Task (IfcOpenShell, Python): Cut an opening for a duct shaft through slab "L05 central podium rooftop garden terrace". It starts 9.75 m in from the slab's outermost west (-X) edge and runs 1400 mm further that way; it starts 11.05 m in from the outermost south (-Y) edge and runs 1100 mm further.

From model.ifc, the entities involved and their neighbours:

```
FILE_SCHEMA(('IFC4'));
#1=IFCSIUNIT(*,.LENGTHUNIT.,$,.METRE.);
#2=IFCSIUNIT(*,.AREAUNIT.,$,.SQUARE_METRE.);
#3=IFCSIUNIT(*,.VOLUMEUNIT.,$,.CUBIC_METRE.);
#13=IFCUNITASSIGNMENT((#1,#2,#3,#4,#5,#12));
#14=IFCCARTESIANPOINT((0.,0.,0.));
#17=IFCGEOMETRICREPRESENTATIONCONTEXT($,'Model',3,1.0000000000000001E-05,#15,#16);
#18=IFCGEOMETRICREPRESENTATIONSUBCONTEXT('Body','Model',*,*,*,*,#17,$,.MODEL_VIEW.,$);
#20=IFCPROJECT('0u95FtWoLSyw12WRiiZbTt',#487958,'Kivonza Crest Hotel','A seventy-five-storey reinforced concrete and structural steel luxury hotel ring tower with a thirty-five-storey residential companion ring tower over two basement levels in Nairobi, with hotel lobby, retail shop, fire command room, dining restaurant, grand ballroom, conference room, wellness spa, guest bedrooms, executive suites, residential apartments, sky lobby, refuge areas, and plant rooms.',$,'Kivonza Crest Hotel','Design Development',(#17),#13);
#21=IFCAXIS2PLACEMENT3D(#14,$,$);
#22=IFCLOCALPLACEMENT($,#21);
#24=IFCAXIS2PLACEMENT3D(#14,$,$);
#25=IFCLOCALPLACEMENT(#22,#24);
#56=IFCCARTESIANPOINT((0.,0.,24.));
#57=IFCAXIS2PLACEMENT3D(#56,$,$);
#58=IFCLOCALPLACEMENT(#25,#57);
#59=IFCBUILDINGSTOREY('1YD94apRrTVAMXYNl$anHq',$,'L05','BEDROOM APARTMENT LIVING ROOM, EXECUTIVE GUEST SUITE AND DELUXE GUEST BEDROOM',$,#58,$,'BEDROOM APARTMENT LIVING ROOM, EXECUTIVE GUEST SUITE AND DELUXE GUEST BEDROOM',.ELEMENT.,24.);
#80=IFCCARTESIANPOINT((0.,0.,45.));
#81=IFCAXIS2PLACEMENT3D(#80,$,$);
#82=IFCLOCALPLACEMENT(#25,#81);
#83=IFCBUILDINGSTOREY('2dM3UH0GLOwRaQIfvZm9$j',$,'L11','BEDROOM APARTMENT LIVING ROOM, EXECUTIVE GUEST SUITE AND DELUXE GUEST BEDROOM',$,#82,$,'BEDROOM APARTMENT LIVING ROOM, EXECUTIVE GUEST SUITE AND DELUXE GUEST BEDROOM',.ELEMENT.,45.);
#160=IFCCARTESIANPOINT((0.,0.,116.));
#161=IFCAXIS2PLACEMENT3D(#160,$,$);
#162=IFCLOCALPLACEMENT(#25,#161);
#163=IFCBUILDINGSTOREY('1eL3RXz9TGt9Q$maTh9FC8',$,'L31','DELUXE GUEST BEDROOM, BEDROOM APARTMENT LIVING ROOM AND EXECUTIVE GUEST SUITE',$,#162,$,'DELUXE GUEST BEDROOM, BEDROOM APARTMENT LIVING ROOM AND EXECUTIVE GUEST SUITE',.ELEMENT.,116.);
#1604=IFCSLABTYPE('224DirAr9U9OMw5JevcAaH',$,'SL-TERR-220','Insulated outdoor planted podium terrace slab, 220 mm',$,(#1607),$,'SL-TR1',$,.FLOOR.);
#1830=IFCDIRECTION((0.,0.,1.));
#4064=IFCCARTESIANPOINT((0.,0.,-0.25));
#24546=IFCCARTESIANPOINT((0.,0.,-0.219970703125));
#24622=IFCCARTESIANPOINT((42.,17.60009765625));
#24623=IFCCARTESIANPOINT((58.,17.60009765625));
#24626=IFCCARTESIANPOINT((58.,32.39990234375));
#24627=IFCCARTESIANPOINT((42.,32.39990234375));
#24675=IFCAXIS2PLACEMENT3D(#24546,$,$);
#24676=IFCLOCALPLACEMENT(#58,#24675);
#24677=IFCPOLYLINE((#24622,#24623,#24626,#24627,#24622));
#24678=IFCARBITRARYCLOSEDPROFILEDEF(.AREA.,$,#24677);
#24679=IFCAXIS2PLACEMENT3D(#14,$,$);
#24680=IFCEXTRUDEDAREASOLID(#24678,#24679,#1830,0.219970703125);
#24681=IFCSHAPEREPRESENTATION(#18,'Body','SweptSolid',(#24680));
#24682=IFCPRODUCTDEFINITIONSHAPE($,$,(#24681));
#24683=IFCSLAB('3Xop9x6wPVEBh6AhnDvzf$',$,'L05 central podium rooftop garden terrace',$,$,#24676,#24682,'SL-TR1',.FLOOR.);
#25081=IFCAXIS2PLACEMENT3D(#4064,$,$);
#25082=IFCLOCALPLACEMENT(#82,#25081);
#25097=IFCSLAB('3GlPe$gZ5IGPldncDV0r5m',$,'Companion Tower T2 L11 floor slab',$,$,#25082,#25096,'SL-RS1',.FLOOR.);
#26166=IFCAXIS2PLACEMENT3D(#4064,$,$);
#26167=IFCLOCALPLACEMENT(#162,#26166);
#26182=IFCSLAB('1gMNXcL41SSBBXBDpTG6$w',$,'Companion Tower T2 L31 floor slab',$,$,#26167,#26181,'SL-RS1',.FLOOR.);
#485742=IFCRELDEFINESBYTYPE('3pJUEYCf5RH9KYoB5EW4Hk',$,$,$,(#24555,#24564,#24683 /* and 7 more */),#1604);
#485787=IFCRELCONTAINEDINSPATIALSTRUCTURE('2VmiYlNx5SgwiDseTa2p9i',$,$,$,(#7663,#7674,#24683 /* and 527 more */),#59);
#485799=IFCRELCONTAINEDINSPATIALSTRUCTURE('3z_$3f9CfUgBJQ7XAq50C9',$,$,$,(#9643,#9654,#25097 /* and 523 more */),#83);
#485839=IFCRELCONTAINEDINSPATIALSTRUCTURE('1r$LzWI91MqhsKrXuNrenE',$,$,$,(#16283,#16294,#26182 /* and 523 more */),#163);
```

```python
import numpy as np
import ifcopenshell
import ifcopenshell.api.feature
import ifcopenshell.api.geometry
import ifcopenshell.api.root
import ifcopenshell.geom
import ifcopenshell.util.placement
import ifcopenshell.util.representation
import ifcopenshell.util.shape
import ifcopenshell.util.unit

model = ifcopenshell.open("model.ifc")
unit_scale = ifcopenshell.util.unit.calculate_unit_scale(model)
settings = ifcopenshell.geom.settings()


def volume(element):
    """Net volume in cubic metres, openings subtracted."""
    shape = ifcopenshell.geom.create_shape(settings, element)
    return ifcopenshell.util.shape.get_volume(shape.geometry)


slab = model.by_guid("3Xop9x6wPVEBh6AhnDvzf$")
before = volume(slab)

# Extent in the slab's own axes, in metres. The edges named are its -X and -Y sides.
slab_shape = ifcopenshell.geom.create_shape(settings, slab)
vertices = ifcopenshell.util.shape.get_vertices(slab_shape.geometry)
x_min, y_min, bottom = vertices.min(axis=0)
top = vertices[:, 2].max()

opening = ifcopenshell.api.root.create_entity(model, ifc_class="IfcOpeningElement", name="Duct shaft opening", predefined_type="OPENING")
context = ifcopenshell.util.representation.get_context(model, "Model", "Body", "MODEL_VIEW")
width, depth = 1.4, 1.1
outline = [(0.0, 0.0), (width, 0.0), (width, depth), (0.0, depth), (0.0, 0.0)]
# Overshoot both faces by 50 mm so the cut is clean.
shape = ifcopenshell.api.geometry.add_slab_representation(
    model, context=context, depth=top - bottom + 0.1, polyline=outline
)
ifcopenshell.api.geometry.assign_representation(model, product=opening, representation=shape)

matrix = ifcopenshell.util.placement.get_local_placement(slab.ObjectPlacement)
matrix[:, 3] = matrix @ np.append(np.array([x_min + 9.75, y_min + 11.05, bottom - 0.05]) / unit_scale, 1.0)
ifcopenshell.api.geometry.edit_object_placement(model, product=opening, matrix=matrix, is_si=False)
ifcopenshell.api.feature.add_feature(model, feature=opening, element=slab)

after = volume(slab)

print(f"slab volume {before:.3f} -> {after:.3f} m3")

model.write("model_v2.ifc")
```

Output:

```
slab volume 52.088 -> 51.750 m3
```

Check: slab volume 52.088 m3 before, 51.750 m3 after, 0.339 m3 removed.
